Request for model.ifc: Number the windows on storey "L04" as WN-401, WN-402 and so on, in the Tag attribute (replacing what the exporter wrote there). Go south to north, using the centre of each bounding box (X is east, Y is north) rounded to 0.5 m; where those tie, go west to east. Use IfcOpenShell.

First a look at what the model holds.

```python
import ifcopenshell
import ifcopenshell.util.element
import ifcopenshell.util.placement

model = ifcopenshell.open("model.ifc")
print(model.schema)
storey = next(s for s in model.by_type("IfcBuildingStorey") if s.Name == "L04")
windows = [e for e in ifcopenshell.util.element.get_decomposition(storey) if e.is_a("IfcWindow")]
for e in sorted(windows, key=lambda e: e.id()):
    origin = ifcopenshell.util.placement.get_local_placement(e.ObjectPlacement)[:3, 3]
    print(e.id(), e.Tag, e.Name, origin.round(2) + 0.0, sep=" | ")
```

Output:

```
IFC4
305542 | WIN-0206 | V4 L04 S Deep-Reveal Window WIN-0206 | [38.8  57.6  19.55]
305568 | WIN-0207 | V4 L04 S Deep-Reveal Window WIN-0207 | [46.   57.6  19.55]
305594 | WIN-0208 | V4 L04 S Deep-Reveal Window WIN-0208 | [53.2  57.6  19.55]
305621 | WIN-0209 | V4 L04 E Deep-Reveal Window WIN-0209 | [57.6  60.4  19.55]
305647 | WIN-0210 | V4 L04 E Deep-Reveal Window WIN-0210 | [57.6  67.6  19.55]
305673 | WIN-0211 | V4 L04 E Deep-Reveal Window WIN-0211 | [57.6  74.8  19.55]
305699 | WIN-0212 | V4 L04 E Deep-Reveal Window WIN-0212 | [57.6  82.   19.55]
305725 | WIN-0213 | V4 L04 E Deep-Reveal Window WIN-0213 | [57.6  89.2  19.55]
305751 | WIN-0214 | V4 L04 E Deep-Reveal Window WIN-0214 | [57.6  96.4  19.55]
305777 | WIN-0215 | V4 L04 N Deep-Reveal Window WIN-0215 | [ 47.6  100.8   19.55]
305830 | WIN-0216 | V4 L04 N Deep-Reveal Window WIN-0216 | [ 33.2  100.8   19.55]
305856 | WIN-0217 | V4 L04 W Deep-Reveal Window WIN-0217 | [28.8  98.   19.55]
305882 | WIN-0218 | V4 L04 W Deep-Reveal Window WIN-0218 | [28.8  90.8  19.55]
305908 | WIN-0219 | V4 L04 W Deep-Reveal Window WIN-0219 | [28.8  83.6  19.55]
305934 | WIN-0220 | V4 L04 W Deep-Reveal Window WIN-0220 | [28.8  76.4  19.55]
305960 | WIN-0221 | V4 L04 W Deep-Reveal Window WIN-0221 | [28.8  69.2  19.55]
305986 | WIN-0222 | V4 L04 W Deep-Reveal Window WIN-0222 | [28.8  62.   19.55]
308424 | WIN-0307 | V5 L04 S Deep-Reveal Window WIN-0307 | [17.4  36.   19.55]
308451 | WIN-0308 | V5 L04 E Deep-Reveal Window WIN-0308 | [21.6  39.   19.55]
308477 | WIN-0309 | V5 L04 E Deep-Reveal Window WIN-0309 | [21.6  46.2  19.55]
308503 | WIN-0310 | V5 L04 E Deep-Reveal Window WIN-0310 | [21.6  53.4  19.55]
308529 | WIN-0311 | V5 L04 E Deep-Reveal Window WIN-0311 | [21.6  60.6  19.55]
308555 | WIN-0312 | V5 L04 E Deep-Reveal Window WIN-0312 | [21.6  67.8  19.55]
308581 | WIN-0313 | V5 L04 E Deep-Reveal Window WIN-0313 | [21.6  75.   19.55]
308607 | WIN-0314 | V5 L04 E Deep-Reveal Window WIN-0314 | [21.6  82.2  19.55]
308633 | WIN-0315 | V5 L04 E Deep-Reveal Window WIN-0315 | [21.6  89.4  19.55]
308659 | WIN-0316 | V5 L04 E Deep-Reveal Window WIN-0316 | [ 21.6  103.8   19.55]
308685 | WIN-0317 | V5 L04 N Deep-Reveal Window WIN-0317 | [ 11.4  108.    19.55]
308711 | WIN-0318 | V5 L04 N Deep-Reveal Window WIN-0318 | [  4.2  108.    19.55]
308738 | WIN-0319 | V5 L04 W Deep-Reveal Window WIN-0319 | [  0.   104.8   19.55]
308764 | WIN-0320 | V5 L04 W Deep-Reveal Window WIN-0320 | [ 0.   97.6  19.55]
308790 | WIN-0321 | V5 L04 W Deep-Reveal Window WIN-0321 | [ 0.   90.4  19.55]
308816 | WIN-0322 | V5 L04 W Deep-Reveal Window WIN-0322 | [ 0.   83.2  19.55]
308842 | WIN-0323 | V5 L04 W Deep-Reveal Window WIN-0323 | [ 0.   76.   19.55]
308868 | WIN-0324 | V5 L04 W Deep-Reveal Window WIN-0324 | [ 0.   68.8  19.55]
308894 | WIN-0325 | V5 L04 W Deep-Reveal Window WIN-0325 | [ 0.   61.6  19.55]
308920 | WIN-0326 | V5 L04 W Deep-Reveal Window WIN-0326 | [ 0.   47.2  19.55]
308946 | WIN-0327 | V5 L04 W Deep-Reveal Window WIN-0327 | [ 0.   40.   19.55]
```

```python
import ifcopenshell
import ifcopenshell.geom
import ifcopenshell.util.element
import ifcopenshell.util.shape

model = ifcopenshell.open("model.ifc")
settings = ifcopenshell.geom.settings()
settings.set("use-world-coords", True)


def centre(element):
    shape = ifcopenshell.geom.create_shape(settings, element)
    return ifcopenshell.util.shape.get_bbox_centroid(shape.geometry)


storey = next(s for s in model.by_type("IfcBuildingStorey") if s.Name == "L04")
windows = [e for e in ifcopenshell.util.element.get_decomposition(storey) if e.is_a("IfcWindow")]

# Insertion points can sit at a corner or the storey origin, so sort by the geometry (in metres).
centres = {e: centre(e) for e in windows}
windows.sort(key=lambda e: (round(centres[e][1] / 0.5), centres[e][0]))

for i, e in enumerate(windows, start=1):
    number = f"WN-4{i:02d}"
    e.Tag = number
    print(e.id(), number)

model.write("model_updated.ifc")
```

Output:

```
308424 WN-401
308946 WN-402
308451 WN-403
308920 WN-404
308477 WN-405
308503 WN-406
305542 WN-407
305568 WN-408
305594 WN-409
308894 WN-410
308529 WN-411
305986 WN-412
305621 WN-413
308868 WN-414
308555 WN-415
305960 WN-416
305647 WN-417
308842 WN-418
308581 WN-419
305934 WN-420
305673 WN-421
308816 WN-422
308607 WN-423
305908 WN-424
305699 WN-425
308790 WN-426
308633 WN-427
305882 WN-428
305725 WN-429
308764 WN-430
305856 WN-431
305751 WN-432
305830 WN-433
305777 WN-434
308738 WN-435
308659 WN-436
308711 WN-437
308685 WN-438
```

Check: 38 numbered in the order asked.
